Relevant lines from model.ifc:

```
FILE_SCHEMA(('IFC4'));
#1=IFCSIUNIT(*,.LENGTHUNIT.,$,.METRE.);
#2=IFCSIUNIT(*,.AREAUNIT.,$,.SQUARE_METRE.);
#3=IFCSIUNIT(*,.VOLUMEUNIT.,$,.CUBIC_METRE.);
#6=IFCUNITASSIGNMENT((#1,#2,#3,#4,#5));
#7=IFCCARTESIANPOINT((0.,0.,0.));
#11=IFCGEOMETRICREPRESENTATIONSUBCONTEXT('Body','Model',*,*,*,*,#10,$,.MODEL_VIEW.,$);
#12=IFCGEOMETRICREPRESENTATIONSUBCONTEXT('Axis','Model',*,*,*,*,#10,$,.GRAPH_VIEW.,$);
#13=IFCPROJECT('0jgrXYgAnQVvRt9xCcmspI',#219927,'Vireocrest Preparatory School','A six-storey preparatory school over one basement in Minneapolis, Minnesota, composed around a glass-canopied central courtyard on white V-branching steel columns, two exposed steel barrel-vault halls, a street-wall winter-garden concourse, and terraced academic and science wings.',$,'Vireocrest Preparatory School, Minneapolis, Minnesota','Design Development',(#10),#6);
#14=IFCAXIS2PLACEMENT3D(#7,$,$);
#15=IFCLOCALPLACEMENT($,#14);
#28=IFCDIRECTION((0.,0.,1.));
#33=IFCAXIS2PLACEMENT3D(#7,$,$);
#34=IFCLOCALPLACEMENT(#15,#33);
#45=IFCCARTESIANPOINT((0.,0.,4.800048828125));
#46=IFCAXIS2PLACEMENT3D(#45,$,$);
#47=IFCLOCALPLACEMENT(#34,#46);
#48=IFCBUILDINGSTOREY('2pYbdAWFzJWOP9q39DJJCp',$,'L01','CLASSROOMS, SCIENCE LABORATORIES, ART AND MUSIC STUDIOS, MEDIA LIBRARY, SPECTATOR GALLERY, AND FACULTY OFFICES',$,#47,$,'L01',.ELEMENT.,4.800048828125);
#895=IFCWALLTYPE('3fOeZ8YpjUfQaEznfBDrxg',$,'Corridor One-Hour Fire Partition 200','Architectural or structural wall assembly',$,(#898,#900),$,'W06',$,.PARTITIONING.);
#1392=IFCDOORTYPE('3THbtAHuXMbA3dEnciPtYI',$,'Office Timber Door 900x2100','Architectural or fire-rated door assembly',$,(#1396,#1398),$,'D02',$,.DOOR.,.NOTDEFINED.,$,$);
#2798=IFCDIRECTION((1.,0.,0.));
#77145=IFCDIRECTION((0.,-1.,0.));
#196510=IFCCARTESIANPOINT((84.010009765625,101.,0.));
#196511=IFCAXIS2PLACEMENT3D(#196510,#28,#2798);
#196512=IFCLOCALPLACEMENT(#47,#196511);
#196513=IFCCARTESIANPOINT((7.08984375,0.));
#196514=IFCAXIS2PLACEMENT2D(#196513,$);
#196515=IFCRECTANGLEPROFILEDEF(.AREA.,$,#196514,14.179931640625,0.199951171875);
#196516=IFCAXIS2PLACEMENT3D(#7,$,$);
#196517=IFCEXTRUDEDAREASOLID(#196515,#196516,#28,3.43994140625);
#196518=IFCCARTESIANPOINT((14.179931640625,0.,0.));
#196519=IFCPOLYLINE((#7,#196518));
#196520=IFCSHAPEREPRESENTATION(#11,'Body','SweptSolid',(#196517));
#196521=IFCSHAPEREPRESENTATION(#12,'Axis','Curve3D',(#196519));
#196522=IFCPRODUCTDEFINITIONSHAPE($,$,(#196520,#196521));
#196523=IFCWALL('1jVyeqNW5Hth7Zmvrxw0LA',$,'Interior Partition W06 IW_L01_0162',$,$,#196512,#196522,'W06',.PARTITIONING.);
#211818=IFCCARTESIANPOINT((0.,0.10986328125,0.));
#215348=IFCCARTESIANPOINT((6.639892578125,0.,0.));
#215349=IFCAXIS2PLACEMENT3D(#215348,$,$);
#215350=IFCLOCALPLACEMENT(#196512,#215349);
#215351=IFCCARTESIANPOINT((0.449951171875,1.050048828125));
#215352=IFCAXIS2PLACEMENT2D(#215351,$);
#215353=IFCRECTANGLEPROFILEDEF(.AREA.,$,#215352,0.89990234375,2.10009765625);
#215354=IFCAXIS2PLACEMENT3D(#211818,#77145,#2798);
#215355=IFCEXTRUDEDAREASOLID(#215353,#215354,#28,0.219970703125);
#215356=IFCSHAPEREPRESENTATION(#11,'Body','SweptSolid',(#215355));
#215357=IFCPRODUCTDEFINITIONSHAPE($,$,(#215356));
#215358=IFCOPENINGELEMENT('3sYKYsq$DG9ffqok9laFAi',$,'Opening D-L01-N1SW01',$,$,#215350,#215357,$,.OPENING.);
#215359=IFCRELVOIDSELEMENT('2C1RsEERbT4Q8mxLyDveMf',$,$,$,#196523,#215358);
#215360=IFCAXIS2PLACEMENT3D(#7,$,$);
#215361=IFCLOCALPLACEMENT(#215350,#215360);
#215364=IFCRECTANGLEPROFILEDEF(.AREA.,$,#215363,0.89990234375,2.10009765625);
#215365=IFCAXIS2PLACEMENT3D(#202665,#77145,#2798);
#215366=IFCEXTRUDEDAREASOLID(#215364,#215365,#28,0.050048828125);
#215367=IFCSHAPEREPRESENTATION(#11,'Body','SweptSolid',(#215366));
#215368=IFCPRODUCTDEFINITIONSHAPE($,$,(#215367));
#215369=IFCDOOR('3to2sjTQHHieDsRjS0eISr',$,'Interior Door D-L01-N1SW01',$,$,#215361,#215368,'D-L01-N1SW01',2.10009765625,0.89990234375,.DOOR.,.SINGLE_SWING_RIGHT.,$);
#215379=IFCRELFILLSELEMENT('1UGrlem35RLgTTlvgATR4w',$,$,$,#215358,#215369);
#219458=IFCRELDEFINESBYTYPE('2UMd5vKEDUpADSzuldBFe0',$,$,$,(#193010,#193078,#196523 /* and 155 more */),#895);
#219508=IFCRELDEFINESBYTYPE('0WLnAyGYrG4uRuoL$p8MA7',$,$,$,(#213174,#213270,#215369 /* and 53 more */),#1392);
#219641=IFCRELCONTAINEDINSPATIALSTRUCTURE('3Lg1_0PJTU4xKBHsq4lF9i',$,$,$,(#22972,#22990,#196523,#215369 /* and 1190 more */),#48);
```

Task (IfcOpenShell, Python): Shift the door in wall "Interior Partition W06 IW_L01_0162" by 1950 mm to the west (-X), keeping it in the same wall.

```python
import ifcopenshell
import ifcopenshell.api.geometry
import ifcopenshell.util.placement
import ifcopenshell.util.unit

model = ifcopenshell.open("model.ifc")
unit_scale = ifcopenshell.util.unit.calculate_unit_scale(model)

door = model.by_guid("3to2sjTQHHieDsRjS0eISr")
opening = door.FillsVoids[0].RelatingOpeningElement
wall = opening.VoidsElements[0].RelatingBuildingElement

wall_matrix = ifcopenshell.util.placement.get_local_placement(wall.ObjectPlacement)
shift = wall_matrix[:3, 0] * -1.95 / unit_scale
before = ifcopenshell.util.placement.get_local_placement(door.ObjectPlacement)[:3, 3].copy()

# The door is placed relative to its opening, so it follows when the opening moves.
matrix = ifcopenshell.util.placement.get_local_placement(opening.ObjectPlacement)
matrix[:3, 3] += shift
ifcopenshell.api.geometry.edit_object_placement(
    model, product=opening, matrix=matrix, is_si=False, should_transform_children=True
)

after = ifcopenshell.util.placement.get_local_placement(door.ObjectPlacement)[:3, 3]
print("door moved by", (after - before).round(3) + 0.0)

model.write("model-out.ifc")
```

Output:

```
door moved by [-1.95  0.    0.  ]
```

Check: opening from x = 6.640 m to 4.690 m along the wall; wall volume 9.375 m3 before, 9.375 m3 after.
